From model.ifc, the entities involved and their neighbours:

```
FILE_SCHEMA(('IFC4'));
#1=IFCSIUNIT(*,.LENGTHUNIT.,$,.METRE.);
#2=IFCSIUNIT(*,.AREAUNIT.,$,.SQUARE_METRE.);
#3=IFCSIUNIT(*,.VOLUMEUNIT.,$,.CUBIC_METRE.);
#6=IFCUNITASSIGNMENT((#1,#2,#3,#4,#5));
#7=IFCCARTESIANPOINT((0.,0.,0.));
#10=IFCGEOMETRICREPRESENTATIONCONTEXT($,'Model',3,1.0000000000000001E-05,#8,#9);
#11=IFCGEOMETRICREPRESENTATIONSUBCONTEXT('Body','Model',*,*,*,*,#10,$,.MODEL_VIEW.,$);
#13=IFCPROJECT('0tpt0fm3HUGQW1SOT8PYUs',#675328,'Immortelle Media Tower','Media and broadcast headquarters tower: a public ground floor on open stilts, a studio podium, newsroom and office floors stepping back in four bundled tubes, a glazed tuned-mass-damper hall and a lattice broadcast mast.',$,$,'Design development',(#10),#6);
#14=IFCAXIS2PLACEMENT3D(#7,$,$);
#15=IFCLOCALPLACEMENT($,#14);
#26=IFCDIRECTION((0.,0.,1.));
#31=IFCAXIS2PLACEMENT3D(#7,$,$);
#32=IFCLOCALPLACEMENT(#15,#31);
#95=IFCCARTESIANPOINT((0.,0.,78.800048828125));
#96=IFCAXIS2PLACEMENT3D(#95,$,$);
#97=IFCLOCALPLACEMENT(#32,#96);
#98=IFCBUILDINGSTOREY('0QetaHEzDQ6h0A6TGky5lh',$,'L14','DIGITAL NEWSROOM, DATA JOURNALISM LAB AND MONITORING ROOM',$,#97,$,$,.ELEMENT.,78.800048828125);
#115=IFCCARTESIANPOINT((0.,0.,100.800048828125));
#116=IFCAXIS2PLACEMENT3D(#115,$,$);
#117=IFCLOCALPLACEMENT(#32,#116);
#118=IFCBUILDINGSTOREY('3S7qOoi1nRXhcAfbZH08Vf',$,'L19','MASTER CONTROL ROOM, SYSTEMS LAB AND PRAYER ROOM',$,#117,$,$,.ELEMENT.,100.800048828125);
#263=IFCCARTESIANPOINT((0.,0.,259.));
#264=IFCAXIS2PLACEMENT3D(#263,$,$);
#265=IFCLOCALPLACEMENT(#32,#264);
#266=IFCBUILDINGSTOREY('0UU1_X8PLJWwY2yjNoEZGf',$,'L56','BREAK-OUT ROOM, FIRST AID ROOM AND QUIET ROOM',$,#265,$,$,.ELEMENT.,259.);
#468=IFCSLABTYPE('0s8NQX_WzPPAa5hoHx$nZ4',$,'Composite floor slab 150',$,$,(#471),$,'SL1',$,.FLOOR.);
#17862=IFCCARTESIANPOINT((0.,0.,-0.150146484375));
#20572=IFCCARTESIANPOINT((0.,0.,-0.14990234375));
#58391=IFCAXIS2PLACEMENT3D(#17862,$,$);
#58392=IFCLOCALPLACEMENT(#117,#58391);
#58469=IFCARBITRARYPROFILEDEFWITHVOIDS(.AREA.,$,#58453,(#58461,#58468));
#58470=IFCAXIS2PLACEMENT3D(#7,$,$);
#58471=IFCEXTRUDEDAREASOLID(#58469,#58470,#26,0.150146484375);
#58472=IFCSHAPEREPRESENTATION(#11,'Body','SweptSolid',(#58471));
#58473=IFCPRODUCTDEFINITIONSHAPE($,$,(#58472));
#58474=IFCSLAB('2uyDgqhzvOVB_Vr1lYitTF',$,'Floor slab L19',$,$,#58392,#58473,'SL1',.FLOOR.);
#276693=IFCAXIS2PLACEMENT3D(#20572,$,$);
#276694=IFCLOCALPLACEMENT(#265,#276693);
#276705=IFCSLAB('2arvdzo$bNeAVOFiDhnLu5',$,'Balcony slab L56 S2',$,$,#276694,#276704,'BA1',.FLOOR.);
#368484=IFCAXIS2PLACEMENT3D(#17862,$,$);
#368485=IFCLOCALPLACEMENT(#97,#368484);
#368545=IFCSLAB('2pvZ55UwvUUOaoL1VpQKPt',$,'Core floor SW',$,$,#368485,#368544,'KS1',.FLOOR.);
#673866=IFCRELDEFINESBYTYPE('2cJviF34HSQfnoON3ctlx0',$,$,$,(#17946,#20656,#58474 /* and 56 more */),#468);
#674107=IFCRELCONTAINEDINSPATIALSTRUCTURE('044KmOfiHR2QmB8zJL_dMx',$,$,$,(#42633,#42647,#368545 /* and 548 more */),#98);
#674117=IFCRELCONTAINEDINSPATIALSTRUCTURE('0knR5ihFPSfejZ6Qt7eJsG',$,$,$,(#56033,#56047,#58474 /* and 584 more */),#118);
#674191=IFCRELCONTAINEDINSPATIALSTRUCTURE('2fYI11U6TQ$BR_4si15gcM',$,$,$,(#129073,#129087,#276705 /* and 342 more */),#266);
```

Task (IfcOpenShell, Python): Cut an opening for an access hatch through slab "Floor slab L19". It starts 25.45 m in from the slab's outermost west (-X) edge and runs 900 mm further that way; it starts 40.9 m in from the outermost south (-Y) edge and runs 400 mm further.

```python
import numpy as np
import ifcopenshell
import ifcopenshell.api.feature
import ifcopenshell.api.geometry
import ifcopenshell.api.root
import ifcopenshell.geom
import ifcopenshell.util.placement
import ifcopenshell.util.representation
import ifcopenshell.util.shape
import ifcopenshell.util.unit

model = ifcopenshell.open("model.ifc")
unit_scale = ifcopenshell.util.unit.calculate_unit_scale(model)
settings = ifcopenshell.geom.settings()


def volume(element):
    """Net volume in cubic metres, openings subtracted."""
    shape = ifcopenshell.geom.create_shape(settings, element)
    return ifcopenshell.util.shape.get_volume(shape.geometry)


slab = model.by_guid("2uyDgqhzvOVB_Vr1lYitTF")
before = volume(slab)

# Extent in the slab's own axes, in metres. The edges named are its -X and -Y sides.
slab_shape = ifcopenshell.geom.create_shape(settings, slab)
vertices = ifcopenshell.util.shape.get_vertices(slab_shape.geometry)
x_min, y_min, bottom = vertices.min(axis=0)
top = vertices[:, 2].max()

opening = ifcopenshell.api.root.create_entity(model, ifc_class="IfcOpeningElement", name="Access hatch opening", predefined_type="OPENING")
context = ifcopenshell.util.representation.get_context(model, "Model", "Body", "MODEL_VIEW")
width, depth = 0.9, 0.4
outline = [(0.0, 0.0), (width, 0.0), (width, depth), (0.0, depth), (0.0, 0.0)]
# Overshoot both faces by 50 mm so the cut is clean.
shape = ifcopenshell.api.geometry.add_slab_representation(
    model, context=context, depth=top - bottom + 0.1, polyline=outline
)
ifcopenshell.api.geometry.assign_representation(model, product=opening, representation=shape)

matrix = ifcopenshell.util.placement.get_local_placement(slab.ObjectPlacement)
matrix[:, 3] = matrix @ np.append(np.array([x_min + 25.45, y_min + 40.9, bottom - 0.05]) / unit_scale, 1.0)
ifcopenshell.api.geometry.edit_object_placement(model, product=opening, matrix=matrix, is_si=False)
ifcopenshell.api.feature.add_feature(model, feature=opening, element=slab)

after = volume(slab)

print(f"slab volume {before:.3f} -> {after:.3f} m3")

model.write("model_edited.ifc")
```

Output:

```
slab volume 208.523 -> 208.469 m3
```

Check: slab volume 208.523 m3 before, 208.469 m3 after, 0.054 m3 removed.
